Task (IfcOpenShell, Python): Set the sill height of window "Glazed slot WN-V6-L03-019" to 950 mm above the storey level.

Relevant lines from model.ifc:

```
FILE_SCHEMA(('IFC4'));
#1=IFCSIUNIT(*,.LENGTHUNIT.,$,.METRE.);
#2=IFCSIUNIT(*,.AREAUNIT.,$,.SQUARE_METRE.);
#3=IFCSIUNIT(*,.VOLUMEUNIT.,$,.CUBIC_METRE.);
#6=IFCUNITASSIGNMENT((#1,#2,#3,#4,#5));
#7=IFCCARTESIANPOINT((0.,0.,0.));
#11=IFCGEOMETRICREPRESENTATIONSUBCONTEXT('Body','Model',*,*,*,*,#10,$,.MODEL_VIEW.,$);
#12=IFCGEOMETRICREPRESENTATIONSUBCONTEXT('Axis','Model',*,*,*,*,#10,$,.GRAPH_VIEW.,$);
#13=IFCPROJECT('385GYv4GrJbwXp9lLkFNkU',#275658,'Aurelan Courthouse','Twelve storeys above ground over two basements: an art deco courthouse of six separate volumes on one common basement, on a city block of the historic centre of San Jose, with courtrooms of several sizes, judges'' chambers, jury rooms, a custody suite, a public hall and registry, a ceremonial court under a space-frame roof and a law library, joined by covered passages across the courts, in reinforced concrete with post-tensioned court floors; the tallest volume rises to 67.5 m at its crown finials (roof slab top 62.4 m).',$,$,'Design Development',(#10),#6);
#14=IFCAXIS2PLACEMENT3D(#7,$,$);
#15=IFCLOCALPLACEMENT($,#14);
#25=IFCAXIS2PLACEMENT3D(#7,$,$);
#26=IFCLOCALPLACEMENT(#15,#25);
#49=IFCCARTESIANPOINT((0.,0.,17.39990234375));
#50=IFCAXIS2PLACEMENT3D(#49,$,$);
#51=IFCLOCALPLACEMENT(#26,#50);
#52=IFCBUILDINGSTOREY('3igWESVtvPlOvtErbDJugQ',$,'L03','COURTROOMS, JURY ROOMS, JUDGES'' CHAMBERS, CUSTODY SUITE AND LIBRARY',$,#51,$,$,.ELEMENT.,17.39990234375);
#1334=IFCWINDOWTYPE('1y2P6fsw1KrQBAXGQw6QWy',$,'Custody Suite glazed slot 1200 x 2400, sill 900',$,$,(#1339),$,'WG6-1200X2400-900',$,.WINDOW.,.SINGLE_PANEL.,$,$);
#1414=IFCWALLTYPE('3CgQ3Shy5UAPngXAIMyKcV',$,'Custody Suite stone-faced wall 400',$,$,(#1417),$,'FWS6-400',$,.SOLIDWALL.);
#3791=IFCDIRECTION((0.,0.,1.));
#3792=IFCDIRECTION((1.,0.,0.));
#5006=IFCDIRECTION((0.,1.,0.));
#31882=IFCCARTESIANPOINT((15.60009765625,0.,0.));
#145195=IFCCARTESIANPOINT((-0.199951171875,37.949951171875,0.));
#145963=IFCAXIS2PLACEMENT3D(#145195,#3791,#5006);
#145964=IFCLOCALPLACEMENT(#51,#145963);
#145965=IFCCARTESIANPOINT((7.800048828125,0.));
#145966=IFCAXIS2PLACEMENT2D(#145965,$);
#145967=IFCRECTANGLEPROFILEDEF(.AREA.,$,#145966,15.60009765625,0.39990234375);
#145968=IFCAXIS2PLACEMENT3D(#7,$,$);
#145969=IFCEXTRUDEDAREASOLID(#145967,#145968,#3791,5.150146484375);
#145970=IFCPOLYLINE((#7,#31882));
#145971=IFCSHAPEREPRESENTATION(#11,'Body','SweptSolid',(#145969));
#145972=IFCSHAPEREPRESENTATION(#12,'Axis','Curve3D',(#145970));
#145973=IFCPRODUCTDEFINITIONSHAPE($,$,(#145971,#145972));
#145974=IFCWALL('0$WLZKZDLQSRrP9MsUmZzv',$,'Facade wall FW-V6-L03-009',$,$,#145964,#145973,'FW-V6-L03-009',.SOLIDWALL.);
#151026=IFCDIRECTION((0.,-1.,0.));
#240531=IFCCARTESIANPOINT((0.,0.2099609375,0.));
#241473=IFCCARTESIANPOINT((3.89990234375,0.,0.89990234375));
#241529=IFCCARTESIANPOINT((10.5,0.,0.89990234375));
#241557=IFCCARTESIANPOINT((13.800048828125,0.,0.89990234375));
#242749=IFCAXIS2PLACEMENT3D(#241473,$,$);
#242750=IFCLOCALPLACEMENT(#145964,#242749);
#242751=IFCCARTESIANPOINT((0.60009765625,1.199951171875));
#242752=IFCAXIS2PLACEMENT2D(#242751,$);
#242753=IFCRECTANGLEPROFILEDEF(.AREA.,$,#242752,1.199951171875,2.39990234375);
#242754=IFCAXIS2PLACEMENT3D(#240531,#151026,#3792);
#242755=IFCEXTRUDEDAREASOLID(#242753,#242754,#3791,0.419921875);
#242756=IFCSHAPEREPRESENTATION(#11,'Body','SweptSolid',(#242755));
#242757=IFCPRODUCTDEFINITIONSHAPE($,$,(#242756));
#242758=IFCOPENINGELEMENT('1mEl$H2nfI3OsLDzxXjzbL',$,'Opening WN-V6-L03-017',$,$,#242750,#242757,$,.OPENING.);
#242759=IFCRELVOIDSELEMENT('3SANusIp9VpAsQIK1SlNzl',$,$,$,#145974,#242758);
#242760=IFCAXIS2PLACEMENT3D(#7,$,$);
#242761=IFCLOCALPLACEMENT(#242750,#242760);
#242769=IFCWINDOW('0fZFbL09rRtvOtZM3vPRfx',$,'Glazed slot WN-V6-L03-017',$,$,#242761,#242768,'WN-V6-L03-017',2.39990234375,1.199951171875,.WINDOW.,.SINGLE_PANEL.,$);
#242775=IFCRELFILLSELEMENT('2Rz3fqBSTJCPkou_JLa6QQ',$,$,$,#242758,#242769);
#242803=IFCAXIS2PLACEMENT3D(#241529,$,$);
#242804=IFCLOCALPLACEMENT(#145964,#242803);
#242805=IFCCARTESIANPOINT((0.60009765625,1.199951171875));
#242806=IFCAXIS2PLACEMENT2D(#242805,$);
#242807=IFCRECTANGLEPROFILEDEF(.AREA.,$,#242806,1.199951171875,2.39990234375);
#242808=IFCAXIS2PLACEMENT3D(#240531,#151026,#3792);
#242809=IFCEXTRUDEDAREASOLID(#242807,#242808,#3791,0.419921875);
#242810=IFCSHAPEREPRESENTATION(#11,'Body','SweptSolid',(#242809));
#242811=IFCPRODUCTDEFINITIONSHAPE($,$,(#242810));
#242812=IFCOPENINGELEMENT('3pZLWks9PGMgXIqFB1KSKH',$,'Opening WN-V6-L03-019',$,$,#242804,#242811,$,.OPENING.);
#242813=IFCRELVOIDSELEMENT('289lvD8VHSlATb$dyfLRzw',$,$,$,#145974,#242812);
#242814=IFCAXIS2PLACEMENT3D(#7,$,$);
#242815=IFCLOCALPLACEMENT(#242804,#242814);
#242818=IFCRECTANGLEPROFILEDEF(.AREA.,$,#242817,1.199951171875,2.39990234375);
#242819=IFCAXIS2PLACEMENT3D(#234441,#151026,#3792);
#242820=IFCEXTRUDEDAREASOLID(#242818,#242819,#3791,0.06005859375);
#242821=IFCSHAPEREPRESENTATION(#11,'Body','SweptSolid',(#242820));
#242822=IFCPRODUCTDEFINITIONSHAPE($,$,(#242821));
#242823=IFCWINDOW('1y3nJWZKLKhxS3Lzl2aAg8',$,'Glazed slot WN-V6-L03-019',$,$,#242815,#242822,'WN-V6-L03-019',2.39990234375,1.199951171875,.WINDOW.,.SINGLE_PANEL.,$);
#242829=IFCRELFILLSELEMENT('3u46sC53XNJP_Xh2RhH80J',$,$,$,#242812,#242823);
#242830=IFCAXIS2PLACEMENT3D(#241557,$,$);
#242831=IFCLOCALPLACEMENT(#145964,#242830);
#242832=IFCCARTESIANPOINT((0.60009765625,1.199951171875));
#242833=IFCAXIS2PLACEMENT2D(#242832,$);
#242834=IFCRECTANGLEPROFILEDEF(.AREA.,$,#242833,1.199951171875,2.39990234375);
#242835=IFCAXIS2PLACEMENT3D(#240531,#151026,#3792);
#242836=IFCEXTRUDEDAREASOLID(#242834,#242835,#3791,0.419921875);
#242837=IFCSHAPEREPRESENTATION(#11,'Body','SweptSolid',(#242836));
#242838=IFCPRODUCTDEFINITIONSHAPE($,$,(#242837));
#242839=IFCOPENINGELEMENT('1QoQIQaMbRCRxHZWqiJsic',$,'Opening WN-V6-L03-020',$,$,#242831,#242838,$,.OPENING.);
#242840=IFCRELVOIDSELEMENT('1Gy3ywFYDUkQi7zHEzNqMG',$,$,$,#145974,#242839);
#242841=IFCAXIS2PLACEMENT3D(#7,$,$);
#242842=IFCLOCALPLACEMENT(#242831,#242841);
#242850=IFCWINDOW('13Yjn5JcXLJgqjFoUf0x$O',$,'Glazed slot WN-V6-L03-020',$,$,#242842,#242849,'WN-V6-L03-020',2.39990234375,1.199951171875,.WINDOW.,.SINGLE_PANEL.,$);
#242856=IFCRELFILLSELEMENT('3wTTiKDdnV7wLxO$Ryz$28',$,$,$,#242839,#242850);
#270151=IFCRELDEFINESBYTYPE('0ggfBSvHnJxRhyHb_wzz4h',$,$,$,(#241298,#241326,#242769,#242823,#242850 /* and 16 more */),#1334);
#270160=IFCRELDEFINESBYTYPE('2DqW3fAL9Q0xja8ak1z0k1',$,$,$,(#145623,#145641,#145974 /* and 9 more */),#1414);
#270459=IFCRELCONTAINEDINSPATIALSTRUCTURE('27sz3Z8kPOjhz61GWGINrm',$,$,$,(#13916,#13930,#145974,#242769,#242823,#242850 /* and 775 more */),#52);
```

```python
import numpy as np
import ifcopenshell
import ifcopenshell.api.geometry
import ifcopenshell.geom
import ifcopenshell.util.element
import ifcopenshell.util.placement
import ifcopenshell.util.shape
import ifcopenshell.util.unit

model = ifcopenshell.open("model.ifc")
unit_scale = ifcopenshell.util.unit.calculate_unit_scale(model)

window = model.by_guid("1y3nJWZKLKhxS3Lzl2aAg8")
opening = window.FillsVoids[0].RelatingOpeningElement
storey = ifcopenshell.util.element.get_container(window, ifc_class="IfcBuildingStorey")
level = ifcopenshell.util.placement.get_local_placement(storey.ObjectPlacement)[2, 3]

# The opening's origin need not be at the sill, so measure its lowest point.
shape = ifcopenshell.geom.create_shape(ifcopenshell.geom.settings(), opening)
bottom = ifcopenshell.util.shape.get_shape_bottom_elevation(shape, shape.geometry) / unit_scale
dz = level + 0.95 - bottom

shift = np.array([0.0, 0.0, dz])
# The window is placed relative to its opening, so it follows when the opening moves.
matrix = ifcopenshell.util.placement.get_local_placement(opening.ObjectPlacement)
matrix[:3, 3] += shift
ifcopenshell.api.geometry.edit_object_placement(
    model, product=opening, matrix=matrix, is_si=False, should_transform_children=True
)

print(f"moved by {dz * unit_scale:+.3f} m")

model.write("model_rev.ifc")
```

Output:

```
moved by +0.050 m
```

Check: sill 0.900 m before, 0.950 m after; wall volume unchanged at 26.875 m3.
